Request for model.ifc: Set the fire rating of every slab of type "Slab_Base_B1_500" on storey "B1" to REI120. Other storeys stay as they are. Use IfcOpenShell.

First a look at what the model holds.

```python
import ifcopenshell
import ifcopenshell.util.element

model = ifcopenshell.open("model.ifc")
print(model.schema)
storey = next(s for s in model.by_type("IfcBuildingStorey") if s.Name == "B1")
slabs = [e for e in ifcopenshell.util.element.get_decomposition(storey) if e.is_a("IfcSlab")]
seen = {}
for e in slabs:
    element_type = ifcopenshell.util.element.get_type(e)
    key = (element_type.Name if element_type != e and element_type else None, ifcopenshell.util.element.get_pset(e, "Pset_SlabCommon", "FireRating"))
    seen[key] = seen.get(key, 0) + 1
for (name, value), count in sorted(seen.items(), key=str):
    print(count, "x", name, "|", value)
```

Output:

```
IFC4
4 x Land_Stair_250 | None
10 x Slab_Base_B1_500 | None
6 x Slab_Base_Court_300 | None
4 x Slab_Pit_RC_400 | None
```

```python
import ifcopenshell
import ifcopenshell.api.pset
import ifcopenshell.util.element

model = ifcopenshell.open("model.ifc")

storey = next(s for s in model.by_type("IfcBuildingStorey") if s.Name == "B1")
slabs = [e for e in ifcopenshell.util.element.get_decomposition(storey) if e.is_a("IfcSlab")]

count = 0
for e in slabs:
    element_type = ifcopenshell.util.element.get_type(e)
    if element_type in (None, e) or element_type.Name != "Slab_Base_B1_500":
        continue
    # add_pset returns the element's existing set when there is one.
    pset = ifcopenshell.api.pset.add_pset(model, product=e, name="Pset_SlabCommon")
    ifcopenshell.api.pset.edit_pset(model, pset=pset, properties={"FireRating": "REI120"})
    count += 1

print(count, "slabs updated")

model.write("model_rev.ifc")
```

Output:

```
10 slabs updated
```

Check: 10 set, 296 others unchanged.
